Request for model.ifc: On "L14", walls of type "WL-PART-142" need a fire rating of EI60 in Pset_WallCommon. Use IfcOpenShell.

First a look at what the model holds.

```python
import ifcopenshell
import ifcopenshell.util.element

model = ifcopenshell.open("model.ifc")
print(model.schema)
storey = next(s for s in model.by_type("IfcBuildingStorey") if s.Name == "L14")
walls = [e for e in ifcopenshell.util.element.get_decomposition(storey) if e.is_a("IfcWall")]
seen = {}
for e in walls:
    element_type = ifcopenshell.util.element.get_type(e)
    key = (element_type.Name if element_type != e and element_type else None, ifcopenshell.util.element.get_pset(e, "Pset_WallCommon", "FireRating"))
    seen[key] = seen.get(key, 0) + 1
for (name, value), count in sorted(seen.items(), key=str):
    print(count, "x", name, "|", value)
```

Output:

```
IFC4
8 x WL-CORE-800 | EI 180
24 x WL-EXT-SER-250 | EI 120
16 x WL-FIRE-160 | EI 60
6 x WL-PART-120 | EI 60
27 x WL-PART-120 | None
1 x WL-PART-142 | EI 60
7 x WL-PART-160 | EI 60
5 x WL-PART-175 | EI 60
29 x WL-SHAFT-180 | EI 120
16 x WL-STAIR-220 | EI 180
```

```python
import ifcopenshell
import ifcopenshell.api.pset
import ifcopenshell.util.element

model = ifcopenshell.open("model.ifc")

storey = next(s for s in model.by_type("IfcBuildingStorey") if s.Name == "L14")
walls = [e for e in ifcopenshell.util.element.get_decomposition(storey) if e.is_a("IfcWall")]

count = 0
for e in walls:
    element_type = ifcopenshell.util.element.get_type(e)
    if element_type in (None, e) or element_type.Name != "WL-PART-142":
        continue
    found = ifcopenshell.util.element.get_pset(e, "Pset_WallCommon", should_inherit=False)
    if found:
        pset = model.by_id(found["id"])
        if len(ifcopenshell.util.element.get_elements_by_pset(pset)) > 1:
            pset = ifcopenshell.api.pset.unshare_pset(model, products=[e], pset=pset)[0]
    else:
        pset = ifcopenshell.api.pset.add_pset(model, product=e, name="Pset_WallCommon")
    ifcopenshell.api.pset.edit_pset(model, pset=pset, properties={"FireRating": "EI60"})
    count += 1

print(count, "walls updated")

model.write("model_rev.ifc")
```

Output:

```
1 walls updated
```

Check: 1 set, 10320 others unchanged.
